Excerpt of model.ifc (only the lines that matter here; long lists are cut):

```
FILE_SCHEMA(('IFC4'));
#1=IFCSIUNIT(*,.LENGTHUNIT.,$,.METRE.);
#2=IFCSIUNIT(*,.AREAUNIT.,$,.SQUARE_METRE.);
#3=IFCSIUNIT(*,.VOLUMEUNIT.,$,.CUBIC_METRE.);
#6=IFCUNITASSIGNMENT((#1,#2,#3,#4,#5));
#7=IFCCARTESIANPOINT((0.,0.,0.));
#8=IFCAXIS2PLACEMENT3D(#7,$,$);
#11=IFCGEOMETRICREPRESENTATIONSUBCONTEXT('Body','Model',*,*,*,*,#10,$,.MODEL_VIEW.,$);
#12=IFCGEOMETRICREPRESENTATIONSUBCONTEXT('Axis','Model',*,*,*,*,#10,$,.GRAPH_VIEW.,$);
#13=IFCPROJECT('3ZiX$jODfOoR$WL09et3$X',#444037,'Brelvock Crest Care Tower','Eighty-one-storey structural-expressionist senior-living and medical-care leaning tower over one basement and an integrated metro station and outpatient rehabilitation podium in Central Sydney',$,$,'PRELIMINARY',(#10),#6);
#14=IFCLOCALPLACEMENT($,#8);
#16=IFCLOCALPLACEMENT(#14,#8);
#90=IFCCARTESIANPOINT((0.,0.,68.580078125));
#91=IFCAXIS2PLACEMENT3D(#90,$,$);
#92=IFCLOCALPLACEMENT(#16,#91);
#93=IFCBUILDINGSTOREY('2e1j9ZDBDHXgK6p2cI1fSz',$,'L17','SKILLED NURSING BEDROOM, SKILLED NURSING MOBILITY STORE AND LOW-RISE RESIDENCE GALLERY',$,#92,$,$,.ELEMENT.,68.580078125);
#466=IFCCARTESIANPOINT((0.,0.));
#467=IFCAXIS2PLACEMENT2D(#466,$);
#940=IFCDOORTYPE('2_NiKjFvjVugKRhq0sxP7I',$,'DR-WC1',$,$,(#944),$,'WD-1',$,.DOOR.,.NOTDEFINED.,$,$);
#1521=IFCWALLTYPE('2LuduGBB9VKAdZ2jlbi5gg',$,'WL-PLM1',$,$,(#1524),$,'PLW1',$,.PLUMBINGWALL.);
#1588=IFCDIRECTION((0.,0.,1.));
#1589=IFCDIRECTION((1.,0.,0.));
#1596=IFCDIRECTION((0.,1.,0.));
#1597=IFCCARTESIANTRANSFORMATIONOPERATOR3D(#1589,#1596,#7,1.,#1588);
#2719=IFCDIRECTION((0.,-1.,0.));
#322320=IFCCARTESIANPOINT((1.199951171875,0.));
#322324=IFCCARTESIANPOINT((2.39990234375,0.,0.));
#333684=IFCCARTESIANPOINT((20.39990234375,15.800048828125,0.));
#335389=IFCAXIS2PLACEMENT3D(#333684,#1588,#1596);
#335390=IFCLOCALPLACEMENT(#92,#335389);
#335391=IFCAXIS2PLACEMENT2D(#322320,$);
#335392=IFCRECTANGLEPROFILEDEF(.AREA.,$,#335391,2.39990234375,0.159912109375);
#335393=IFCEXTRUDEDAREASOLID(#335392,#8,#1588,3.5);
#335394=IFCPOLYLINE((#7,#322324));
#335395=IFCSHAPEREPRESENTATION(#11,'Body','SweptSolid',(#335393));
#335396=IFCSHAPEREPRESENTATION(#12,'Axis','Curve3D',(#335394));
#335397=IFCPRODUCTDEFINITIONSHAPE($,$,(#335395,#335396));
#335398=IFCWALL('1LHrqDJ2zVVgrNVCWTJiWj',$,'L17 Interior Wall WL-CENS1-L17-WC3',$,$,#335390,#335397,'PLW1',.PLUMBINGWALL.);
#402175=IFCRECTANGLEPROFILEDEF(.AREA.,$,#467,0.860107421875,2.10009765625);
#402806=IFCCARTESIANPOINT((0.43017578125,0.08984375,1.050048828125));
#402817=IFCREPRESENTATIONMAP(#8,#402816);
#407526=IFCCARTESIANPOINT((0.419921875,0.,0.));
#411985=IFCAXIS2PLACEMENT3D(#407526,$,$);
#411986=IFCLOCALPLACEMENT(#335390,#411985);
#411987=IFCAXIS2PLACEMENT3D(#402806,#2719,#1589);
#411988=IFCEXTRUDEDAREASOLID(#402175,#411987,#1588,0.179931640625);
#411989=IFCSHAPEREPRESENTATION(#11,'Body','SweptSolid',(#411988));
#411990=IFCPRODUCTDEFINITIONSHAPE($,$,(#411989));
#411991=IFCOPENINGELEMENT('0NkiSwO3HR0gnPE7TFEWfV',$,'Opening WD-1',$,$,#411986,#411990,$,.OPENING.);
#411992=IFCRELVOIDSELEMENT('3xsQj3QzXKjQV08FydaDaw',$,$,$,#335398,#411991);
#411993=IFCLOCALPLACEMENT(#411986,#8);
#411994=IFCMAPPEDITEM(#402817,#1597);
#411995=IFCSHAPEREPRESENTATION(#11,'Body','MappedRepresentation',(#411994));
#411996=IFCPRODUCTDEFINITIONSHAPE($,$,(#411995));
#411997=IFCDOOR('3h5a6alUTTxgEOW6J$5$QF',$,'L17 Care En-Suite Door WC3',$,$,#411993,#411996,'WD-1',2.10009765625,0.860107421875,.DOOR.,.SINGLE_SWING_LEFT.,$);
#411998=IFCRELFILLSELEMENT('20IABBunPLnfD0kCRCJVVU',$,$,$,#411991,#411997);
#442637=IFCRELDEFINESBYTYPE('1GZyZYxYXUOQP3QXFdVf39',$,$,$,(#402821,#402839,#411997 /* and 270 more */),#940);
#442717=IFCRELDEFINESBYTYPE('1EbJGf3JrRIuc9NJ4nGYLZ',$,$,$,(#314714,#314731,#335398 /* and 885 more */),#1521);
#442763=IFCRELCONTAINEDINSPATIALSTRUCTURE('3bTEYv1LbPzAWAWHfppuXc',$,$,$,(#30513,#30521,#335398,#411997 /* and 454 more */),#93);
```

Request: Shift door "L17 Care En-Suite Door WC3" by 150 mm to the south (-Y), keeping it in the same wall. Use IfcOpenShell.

```python
import ifcopenshell
import ifcopenshell.api.geometry
import ifcopenshell.util.placement

model = ifcopenshell.open("model.ifc")

door = model.by_guid("3h5a6alUTTxgEOW6J$5$QF")
opening = door.FillsVoids[0].RelatingOpeningElement
wall = opening.VoidsElements[0].RelatingBuildingElement

wall_matrix = ifcopenshell.util.placement.get_local_placement(wall.ObjectPlacement)
shift = wall_matrix[:3, 0] * -0.15
before = ifcopenshell.util.placement.get_local_placement(door.ObjectPlacement)[:3, 3].copy()

# The door is placed relative to its opening, so it follows when the opening moves.
matrix = ifcopenshell.util.placement.get_local_placement(opening.ObjectPlacement)
matrix[:3, 3] += shift
ifcopenshell.api.geometry.edit_object_placement(
    model, product=opening, matrix=matrix, is_si=False, should_transform_children=True
)

after = ifcopenshell.util.placement.get_local_placement(door.ObjectPlacement)[:3, 3]
print("door moved by", (after - before).round(3) + 0.0)

model.write("model_edited.ifc")
```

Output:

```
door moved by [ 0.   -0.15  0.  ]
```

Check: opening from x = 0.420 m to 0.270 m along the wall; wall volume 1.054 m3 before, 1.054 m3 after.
